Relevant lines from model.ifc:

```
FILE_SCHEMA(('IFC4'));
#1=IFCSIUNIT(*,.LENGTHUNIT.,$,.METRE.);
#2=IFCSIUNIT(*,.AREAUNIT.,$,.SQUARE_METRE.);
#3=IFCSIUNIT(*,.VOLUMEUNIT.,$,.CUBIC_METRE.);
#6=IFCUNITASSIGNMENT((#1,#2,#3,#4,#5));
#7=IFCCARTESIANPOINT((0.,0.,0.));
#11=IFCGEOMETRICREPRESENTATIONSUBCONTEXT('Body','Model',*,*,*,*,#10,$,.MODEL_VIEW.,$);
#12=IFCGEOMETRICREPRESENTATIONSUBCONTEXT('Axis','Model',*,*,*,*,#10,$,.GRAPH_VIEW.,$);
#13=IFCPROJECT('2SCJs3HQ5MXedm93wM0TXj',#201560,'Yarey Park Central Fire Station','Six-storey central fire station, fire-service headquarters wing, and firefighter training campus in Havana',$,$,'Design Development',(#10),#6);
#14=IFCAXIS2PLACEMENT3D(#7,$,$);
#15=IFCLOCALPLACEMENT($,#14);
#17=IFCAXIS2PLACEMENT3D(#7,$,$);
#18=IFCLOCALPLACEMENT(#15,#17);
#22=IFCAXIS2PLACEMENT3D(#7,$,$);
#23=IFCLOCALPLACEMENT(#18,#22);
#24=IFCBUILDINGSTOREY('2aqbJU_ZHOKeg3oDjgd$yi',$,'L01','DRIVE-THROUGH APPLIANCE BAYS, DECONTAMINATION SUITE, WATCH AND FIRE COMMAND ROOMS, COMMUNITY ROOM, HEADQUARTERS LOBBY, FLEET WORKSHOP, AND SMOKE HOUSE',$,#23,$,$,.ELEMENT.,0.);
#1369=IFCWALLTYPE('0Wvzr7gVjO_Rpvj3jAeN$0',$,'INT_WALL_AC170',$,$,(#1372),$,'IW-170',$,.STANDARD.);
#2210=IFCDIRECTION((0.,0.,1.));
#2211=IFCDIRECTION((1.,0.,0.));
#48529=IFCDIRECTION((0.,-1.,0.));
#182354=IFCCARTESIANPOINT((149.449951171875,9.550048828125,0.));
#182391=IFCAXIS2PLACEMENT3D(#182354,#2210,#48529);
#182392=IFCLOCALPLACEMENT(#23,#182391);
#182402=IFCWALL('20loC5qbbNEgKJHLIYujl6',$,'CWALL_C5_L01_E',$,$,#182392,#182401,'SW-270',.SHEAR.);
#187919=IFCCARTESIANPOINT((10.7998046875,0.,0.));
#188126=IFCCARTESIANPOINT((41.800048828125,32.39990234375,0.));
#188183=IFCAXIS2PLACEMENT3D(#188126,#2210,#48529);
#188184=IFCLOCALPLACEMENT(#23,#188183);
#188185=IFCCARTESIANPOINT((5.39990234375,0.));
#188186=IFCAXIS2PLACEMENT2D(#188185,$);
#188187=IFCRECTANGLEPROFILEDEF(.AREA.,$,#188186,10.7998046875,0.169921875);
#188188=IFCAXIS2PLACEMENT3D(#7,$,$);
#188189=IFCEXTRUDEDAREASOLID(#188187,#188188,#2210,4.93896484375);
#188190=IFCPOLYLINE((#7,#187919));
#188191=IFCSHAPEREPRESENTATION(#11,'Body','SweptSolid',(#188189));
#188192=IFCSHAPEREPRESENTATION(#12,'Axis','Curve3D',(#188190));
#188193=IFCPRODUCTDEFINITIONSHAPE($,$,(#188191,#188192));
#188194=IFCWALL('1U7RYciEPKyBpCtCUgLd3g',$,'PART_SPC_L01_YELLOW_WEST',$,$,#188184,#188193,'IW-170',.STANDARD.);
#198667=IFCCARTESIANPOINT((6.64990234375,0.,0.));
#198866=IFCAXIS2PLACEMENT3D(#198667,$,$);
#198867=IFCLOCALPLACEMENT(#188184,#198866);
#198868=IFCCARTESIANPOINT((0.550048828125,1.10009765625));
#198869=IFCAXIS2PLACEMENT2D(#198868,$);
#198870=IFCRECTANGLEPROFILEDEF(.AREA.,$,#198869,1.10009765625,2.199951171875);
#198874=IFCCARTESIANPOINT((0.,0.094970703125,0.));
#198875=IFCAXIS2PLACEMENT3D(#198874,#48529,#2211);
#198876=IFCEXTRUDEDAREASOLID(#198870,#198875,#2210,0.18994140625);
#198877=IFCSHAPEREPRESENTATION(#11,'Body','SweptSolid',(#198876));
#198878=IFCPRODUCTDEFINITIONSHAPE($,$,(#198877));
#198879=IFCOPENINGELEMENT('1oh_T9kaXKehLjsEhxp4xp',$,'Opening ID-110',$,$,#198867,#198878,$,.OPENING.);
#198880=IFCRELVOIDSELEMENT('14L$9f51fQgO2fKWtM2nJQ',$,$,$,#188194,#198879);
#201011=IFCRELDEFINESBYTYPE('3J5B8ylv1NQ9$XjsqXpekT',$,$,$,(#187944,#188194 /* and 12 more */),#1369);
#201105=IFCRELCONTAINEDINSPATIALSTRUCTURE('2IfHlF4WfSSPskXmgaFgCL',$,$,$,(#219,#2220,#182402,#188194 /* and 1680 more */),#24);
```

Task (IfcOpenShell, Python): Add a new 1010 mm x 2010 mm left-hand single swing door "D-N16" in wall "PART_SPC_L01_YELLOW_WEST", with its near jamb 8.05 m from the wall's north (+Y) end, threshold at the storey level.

```python
import numpy as np
import ifcopenshell
import ifcopenshell.api.feature
import ifcopenshell.api.geometry
import ifcopenshell.api.root
import ifcopenshell.api.spatial
import ifcopenshell.geom
import ifcopenshell.util.element
import ifcopenshell.util.placement
import ifcopenshell.util.representation
import ifcopenshell.util.shape
import ifcopenshell.util.unit

model = ifcopenshell.open("model.ifc")
unit_scale = ifcopenshell.util.unit.calculate_unit_scale(model)
settings = ifcopenshell.geom.settings()


def volume(element):
    """Net volume in cubic metres, openings subtracted."""
    shape = ifcopenshell.geom.create_shape(settings, element)
    return ifcopenshell.util.shape.get_volume(shape.geometry)


wall = model.by_guid("1U7RYciEPKyBpCtCUgLd3g")
storey = ifcopenshell.util.element.get_container(wall, ifc_class="IfcBuildingStorey")
context = ifcopenshell.util.representation.get_context(model, "Model", "Body", "MODEL_VIEW")
before = volume(wall)

width, height, from_end, sill = 1.01, 2.01, 8.05, 0.0  # metres

# The wall runs along its own X axis, and the end named is its -X end.
wall_shape = ifcopenshell.geom.create_shape(settings, wall)
x, y, z = ifcopenshell.util.shape.get_vertices(wall_shape.geometry).T
start = x.min() + from_end
face, thickness = float(y.min()), float(y.max() - y.min())
wall_matrix = ifcopenshell.util.placement.get_local_placement(wall.ObjectPlacement)
level = ifcopenshell.util.placement.get_local_placement(storey.ObjectPlacement)[2, 3]


def in_wall(x, y):
    """Placement at x, y metres in the wall's axes, at sill height."""
    matrix = wall_matrix.copy()
    matrix[:, 3] = wall_matrix @ np.array([x / unit_scale, y / unit_scale, 0.0, 1.0])
    matrix[2, 3] = level + sill / unit_scale
    return matrix


# Opening: a box that overshoots both wall faces by 50 mm.
opening = ifcopenshell.api.root.create_entity(model, ifc_class="IfcOpeningElement", predefined_type="OPENING")
box = ifcopenshell.api.geometry.add_wall_representation(
    model, context=context, length=width, height=height, thickness=thickness + 0.1
)
ifcopenshell.api.geometry.assign_representation(model, product=opening, representation=box)
ifcopenshell.api.geometry.edit_object_placement(model, product=opening, matrix=in_wall(start, face - 0.05), is_si=False)
ifcopenshell.api.feature.add_feature(model, feature=opening, element=wall)

door = ifcopenshell.api.root.create_entity(model, ifc_class="IfcDoor", name="D-N16", predefined_type="DOOR")
door.OverallWidth, door.OverallHeight = width / unit_scale, height / unit_scale
door.OperationType = "SINGLE_SWING_LEFT"
body = ifcopenshell.api.geometry.add_door_representation(
    model,
    context=context,
    overall_width=door.OverallWidth,
    overall_height=door.OverallHeight,
    operation_type="SINGLE_SWING_LEFT",
    lining_properties={"LiningDepth": thickness / unit_scale, "ThresholdDepth": thickness / unit_scale},
)
ifcopenshell.api.geometry.assign_representation(model, product=door, representation=body)
ifcopenshell.api.spatial.assign_container(model, products=[door], relating_structure=storey)
ifcopenshell.api.feature.add_filling(model, opening=opening, element=door)

# The lining spans the wall, so the door starts at the wall face.
ifcopenshell.api.geometry.edit_object_placement(model, product=door, matrix=in_wall(start, face), is_si=False)

after = volume(wall)

print(f"wall volume {before:.3f} -> {after:.3f} m3")

model.write("model_updated.ifc")
```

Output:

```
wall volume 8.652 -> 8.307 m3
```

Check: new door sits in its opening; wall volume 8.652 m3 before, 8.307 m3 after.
